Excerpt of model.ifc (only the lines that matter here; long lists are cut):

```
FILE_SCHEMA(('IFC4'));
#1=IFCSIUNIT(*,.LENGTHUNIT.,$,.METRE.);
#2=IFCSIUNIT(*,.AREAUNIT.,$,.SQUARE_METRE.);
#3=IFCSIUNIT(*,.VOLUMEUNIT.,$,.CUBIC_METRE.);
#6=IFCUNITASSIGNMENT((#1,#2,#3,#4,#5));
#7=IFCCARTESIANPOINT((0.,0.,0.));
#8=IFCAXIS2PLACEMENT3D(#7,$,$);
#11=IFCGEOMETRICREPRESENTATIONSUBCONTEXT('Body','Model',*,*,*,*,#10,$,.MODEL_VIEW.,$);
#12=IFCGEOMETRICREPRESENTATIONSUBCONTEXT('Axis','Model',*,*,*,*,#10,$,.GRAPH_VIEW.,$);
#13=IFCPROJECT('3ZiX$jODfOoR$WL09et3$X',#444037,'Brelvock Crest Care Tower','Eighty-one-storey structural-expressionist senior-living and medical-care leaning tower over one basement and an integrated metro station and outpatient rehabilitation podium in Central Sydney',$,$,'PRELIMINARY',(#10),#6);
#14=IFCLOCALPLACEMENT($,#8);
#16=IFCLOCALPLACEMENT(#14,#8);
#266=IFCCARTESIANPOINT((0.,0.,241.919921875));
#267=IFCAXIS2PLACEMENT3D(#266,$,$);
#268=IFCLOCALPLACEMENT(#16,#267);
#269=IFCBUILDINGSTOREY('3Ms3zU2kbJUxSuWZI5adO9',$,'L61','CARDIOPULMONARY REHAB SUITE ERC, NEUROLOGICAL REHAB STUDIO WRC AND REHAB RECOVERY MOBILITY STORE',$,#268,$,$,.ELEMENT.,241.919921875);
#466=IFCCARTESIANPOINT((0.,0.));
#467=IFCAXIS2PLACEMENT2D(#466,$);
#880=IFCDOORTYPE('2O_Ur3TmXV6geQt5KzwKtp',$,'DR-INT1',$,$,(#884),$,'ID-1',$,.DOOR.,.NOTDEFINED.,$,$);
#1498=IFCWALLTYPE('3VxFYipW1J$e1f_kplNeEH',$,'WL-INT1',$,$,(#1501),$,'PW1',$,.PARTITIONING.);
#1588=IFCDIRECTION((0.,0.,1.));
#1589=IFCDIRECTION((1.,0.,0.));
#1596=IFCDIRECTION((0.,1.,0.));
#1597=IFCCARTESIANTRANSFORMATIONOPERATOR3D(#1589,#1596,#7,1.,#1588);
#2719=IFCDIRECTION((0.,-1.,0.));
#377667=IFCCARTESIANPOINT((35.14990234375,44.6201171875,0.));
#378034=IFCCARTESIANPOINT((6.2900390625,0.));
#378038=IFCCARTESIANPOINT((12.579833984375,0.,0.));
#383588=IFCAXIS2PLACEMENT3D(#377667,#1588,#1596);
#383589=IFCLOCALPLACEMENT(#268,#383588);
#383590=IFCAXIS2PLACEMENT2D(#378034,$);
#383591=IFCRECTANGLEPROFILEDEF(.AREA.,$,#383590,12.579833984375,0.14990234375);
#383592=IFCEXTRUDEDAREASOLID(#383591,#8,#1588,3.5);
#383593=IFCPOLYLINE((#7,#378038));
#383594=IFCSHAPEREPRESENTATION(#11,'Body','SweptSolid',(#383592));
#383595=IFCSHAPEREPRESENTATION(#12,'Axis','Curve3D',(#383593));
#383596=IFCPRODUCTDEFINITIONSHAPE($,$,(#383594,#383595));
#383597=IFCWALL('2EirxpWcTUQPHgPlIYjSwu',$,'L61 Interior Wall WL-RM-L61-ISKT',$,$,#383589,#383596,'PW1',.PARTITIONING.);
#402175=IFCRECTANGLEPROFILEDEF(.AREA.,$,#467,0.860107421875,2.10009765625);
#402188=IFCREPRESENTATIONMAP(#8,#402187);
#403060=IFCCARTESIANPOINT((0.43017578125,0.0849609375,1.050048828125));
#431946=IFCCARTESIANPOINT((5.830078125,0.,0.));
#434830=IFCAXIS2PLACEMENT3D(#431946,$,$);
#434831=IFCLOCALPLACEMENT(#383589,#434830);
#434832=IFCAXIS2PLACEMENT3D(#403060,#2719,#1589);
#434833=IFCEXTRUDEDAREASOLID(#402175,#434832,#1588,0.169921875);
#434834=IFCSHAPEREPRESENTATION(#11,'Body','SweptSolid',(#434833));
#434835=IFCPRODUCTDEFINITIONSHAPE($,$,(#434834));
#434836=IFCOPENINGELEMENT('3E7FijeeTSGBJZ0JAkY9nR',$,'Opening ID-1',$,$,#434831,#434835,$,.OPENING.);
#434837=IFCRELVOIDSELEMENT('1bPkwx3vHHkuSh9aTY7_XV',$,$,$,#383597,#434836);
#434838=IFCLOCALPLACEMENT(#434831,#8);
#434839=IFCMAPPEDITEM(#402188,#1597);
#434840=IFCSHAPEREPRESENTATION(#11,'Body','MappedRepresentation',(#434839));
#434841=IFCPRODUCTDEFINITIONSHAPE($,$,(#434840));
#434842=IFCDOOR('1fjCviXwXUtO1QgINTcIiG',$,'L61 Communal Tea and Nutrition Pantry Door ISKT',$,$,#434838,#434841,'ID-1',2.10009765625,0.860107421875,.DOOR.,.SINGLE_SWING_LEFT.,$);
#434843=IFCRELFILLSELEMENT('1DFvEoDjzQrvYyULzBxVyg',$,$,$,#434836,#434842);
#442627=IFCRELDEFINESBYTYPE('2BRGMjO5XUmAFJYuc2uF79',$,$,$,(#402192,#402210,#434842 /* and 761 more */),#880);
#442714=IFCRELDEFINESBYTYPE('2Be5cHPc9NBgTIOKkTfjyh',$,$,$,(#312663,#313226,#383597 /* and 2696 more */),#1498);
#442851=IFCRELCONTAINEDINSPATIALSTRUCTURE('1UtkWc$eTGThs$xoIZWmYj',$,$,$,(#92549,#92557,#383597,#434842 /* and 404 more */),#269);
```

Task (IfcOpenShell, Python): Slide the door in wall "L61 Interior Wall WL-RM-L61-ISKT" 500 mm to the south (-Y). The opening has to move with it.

```python
import ifcopenshell
import ifcopenshell.api.geometry
import ifcopenshell.util.placement

model = ifcopenshell.open("model.ifc")

door = model.by_id(434842)
opening = door.FillsVoids[0].RelatingOpeningElement
wall = opening.VoidsElements[0].RelatingBuildingElement

wall_matrix = ifcopenshell.util.placement.get_local_placement(wall.ObjectPlacement)
shift = wall_matrix[:3, 0] * -0.5
before = ifcopenshell.util.placement.get_local_placement(door.ObjectPlacement)[:3, 3].copy()

# The door is placed relative to its opening, so it follows when the opening moves.
matrix = ifcopenshell.util.placement.get_local_placement(opening.ObjectPlacement)
matrix[:3, 3] += shift
ifcopenshell.api.geometry.edit_object_placement(
    model, product=opening, matrix=matrix, is_si=False, should_transform_children=True
)

after = ifcopenshell.util.placement.get_local_placement(door.ObjectPlacement)[:3, 3]
print("door moved by", (after - before).round(3) + 0.0)

model.write("model_rev.ifc")
```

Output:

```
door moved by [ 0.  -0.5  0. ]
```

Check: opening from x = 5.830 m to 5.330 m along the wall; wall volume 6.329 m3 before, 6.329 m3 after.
